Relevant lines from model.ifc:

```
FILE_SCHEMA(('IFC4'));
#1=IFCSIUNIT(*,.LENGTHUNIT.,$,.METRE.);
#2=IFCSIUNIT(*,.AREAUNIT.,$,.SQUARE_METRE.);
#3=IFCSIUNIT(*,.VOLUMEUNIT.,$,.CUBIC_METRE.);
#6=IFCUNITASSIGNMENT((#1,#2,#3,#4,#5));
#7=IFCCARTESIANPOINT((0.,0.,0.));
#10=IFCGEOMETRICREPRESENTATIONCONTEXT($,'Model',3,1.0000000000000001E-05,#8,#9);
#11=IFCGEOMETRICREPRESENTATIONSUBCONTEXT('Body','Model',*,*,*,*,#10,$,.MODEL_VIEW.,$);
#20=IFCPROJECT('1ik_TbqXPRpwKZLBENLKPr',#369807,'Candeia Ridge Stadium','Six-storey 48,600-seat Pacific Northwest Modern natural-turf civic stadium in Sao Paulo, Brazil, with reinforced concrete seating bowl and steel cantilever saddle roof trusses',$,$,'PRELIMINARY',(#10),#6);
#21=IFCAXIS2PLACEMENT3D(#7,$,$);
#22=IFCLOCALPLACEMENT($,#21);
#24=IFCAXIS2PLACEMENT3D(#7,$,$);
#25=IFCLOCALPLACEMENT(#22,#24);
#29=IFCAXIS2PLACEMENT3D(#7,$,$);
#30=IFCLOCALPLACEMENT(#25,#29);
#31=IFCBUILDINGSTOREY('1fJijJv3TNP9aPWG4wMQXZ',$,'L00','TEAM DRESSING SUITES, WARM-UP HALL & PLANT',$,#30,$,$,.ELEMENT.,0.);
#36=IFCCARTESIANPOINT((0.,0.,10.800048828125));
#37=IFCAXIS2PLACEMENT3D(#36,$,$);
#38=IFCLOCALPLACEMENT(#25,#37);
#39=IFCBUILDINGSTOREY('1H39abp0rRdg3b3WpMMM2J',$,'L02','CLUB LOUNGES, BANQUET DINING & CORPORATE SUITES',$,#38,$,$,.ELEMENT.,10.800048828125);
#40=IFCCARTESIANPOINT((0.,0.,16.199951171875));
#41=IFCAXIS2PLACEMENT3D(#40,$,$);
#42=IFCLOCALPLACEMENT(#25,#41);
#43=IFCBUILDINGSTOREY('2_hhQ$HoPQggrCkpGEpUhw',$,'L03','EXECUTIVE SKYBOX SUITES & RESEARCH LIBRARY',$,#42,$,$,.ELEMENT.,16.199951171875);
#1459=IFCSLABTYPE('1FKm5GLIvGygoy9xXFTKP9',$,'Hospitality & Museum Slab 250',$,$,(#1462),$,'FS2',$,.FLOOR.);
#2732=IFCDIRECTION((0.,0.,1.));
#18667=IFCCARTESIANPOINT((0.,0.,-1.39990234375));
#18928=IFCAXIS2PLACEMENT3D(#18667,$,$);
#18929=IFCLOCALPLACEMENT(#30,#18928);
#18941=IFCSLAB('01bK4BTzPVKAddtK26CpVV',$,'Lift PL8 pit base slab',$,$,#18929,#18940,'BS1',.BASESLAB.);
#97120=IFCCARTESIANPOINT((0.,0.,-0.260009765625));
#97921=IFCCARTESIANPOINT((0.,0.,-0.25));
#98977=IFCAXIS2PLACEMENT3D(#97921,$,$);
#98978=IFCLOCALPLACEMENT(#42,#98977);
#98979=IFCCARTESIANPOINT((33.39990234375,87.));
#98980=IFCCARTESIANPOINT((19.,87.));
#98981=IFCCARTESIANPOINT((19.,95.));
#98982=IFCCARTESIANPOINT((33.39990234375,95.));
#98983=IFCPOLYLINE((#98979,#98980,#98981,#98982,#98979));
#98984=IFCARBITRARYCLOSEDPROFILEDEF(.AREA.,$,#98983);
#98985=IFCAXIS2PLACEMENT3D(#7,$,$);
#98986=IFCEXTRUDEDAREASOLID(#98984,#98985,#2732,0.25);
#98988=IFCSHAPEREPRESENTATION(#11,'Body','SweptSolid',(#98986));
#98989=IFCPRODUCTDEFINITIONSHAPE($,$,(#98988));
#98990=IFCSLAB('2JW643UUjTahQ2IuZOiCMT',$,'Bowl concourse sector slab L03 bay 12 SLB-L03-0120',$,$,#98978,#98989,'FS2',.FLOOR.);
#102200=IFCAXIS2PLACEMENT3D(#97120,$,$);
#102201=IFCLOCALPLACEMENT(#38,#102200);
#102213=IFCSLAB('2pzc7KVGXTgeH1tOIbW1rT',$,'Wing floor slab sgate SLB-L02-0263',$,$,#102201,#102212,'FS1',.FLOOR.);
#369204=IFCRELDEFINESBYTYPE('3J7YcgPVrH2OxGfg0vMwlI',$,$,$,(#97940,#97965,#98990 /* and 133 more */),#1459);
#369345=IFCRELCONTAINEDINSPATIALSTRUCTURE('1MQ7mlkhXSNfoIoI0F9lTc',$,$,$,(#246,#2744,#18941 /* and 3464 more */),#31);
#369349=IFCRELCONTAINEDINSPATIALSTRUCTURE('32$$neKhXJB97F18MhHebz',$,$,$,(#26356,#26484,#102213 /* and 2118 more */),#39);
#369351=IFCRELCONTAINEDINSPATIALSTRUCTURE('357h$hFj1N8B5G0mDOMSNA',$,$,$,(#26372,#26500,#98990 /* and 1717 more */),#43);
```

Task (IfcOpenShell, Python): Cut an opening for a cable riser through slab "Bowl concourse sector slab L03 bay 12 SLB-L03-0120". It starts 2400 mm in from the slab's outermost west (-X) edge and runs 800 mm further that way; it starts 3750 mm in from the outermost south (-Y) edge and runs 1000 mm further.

```python
import numpy as np
import ifcopenshell
import ifcopenshell.api.feature
import ifcopenshell.api.geometry
import ifcopenshell.api.root
import ifcopenshell.geom
import ifcopenshell.util.placement
import ifcopenshell.util.representation
import ifcopenshell.util.shape
import ifcopenshell.util.unit

model = ifcopenshell.open("model.ifc")
unit_scale = ifcopenshell.util.unit.calculate_unit_scale(model)
settings = ifcopenshell.geom.settings()


def volume(element):
    """Net volume in cubic metres, openings subtracted."""
    shape = ifcopenshell.geom.create_shape(settings, element)
    return ifcopenshell.util.shape.get_volume(shape.geometry)


slab = model.by_id(98990)
before = volume(slab)

# Extent in the slab's own axes, in metres. The edges named are its -X and -Y sides.
slab_shape = ifcopenshell.geom.create_shape(settings, slab)
vertices = ifcopenshell.util.shape.get_vertices(slab_shape.geometry)
x_min, y_min, bottom = vertices.min(axis=0)
top = vertices[:, 2].max()

opening = ifcopenshell.api.root.create_entity(model, ifc_class="IfcOpeningElement", name="Cable riser opening", predefined_type="OPENING")
context = ifcopenshell.util.representation.get_context(model, "Model", "Body", "MODEL_VIEW")
width, depth = 0.8, 1
outline = [(0.0, 0.0), (width, 0.0), (width, depth), (0.0, depth), (0.0, 0.0)]
# Overshoot both faces by 50 mm so the cut is clean.
shape = ifcopenshell.api.geometry.add_slab_representation(
    model, context=context, depth=top - bottom + 0.1, polyline=outline
)
ifcopenshell.api.geometry.assign_representation(model, product=opening, representation=shape)

matrix = ifcopenshell.util.placement.get_local_placement(slab.ObjectPlacement)
matrix[:, 3] = matrix @ np.append(np.array([x_min + 2.4, y_min + 3.75, bottom - 0.05]) / unit_scale, 1.0)
ifcopenshell.api.geometry.edit_object_placement(model, product=opening, matrix=matrix, is_si=False)
ifcopenshell.api.feature.add_feature(model, feature=opening, element=slab)

after = volume(slab)

print(f"slab volume {before:.3f} -> {after:.3f} m3")

model.write("model_updated.ifc")
```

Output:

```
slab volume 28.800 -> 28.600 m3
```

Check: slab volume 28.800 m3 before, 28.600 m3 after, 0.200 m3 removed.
